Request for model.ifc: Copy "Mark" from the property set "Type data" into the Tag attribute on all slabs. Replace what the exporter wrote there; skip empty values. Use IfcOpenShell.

First a look at what the model holds.

```python
import ifcopenshell
import ifcopenshell.util.element

model = ifcopenshell.open("model.ifc")
print(model.schema)
slabs = model.by_type("IfcSlab")
print(len(slabs), "slabs")
for e in slabs[:8]:
    source = ifcopenshell.util.element.get_pset(e, "Type data", "Mark")
    target = e.Tag
    print(e.id(), repr(source), repr(target), sep=" | ")
```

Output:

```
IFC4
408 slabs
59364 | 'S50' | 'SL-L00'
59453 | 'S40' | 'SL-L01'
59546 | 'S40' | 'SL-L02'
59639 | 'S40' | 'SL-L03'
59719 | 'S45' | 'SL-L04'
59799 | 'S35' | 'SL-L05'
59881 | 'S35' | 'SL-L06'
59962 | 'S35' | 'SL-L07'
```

```python
import ifcopenshell
import ifcopenshell.util.element

model = ifcopenshell.open("model.ifc")

count = 0
for e in model.by_type("IfcSlab"):
    value = ifcopenshell.util.element.get_pset(e, "Type data", "Mark")
    current = e.Tag
    if not value or not value.strip() or current == value:
        continue
    e.Tag = value
    count += 1

print(count, "slabs updated")

model.write("model_updated.ifc")
```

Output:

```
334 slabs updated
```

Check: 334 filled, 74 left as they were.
